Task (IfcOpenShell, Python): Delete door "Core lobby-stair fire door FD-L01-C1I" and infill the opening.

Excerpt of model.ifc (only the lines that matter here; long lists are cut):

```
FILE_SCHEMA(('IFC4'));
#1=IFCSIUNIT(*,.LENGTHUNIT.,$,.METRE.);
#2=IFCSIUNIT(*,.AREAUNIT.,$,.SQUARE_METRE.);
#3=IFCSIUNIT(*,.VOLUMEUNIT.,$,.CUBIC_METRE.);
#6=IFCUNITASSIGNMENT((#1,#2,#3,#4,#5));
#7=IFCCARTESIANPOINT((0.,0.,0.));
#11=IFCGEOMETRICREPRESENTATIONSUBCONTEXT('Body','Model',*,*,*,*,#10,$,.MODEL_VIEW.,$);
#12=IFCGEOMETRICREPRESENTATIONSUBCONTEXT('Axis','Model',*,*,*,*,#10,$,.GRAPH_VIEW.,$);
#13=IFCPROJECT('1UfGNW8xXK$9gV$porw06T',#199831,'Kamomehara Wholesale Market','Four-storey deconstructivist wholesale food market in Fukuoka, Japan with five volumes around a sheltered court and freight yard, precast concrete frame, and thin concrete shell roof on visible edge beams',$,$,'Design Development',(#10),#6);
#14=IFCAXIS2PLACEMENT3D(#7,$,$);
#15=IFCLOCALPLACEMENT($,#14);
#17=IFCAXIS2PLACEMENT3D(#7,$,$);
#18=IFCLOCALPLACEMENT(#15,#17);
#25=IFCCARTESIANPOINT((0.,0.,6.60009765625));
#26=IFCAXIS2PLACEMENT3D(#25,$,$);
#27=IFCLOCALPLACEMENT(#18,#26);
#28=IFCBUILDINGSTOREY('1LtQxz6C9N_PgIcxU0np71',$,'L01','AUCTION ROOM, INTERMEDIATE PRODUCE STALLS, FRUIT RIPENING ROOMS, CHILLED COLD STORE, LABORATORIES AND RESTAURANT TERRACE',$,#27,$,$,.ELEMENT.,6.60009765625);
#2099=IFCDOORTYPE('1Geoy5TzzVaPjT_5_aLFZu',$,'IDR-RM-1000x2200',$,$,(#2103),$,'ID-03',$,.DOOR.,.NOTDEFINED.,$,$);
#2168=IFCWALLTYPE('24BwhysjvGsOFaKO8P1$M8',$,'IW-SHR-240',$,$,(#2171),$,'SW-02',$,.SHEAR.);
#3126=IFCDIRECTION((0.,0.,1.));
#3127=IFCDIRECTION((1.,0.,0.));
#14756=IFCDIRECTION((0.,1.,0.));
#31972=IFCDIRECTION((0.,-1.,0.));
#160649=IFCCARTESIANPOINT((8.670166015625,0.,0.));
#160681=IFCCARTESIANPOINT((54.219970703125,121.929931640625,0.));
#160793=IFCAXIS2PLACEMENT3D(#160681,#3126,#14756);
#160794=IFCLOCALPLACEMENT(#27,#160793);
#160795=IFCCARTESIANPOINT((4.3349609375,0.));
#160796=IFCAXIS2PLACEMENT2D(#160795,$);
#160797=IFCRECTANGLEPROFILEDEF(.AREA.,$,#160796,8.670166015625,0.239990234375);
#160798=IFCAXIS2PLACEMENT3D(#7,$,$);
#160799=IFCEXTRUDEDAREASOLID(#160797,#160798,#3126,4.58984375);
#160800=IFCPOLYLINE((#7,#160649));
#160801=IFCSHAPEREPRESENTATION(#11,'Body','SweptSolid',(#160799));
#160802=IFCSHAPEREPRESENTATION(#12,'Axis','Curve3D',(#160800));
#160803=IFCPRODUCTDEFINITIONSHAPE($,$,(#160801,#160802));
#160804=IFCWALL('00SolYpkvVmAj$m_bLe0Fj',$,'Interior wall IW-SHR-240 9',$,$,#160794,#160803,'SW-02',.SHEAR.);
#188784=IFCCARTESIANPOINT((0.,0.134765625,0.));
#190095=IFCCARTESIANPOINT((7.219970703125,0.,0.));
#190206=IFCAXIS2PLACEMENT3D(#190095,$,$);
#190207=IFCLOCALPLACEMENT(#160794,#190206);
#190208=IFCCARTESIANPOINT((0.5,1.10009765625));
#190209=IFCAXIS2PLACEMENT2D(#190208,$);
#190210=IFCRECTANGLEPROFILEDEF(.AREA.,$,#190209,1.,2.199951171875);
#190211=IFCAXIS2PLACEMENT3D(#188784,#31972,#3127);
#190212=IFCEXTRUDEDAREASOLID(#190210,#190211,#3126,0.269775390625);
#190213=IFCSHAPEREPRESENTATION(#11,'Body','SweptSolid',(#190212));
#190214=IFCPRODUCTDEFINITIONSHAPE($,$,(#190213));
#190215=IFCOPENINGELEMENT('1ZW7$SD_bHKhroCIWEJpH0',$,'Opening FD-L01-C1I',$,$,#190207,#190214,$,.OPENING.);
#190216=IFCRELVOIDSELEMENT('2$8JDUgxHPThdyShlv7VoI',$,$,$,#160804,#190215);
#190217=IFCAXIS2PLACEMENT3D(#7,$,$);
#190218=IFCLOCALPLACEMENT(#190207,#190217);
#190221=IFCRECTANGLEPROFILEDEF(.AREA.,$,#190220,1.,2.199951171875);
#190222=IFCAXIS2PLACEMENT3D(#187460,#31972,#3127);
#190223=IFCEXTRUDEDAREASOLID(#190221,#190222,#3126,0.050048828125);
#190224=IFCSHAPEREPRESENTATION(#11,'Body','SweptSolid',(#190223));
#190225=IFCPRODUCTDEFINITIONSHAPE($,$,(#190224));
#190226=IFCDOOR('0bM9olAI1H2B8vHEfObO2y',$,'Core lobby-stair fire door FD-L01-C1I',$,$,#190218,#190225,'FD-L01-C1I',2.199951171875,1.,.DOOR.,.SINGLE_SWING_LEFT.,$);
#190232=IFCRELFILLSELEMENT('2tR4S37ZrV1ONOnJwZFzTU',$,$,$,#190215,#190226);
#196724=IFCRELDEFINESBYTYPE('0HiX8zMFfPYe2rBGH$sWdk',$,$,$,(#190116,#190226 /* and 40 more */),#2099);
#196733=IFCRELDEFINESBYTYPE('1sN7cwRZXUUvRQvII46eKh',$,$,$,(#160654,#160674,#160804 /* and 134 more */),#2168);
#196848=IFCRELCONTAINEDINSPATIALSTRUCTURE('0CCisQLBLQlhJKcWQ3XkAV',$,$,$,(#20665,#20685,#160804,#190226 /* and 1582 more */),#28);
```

```python
import ifcopenshell
import ifcopenshell.api.feature
import ifcopenshell.api.root
import ifcopenshell.geom
import ifcopenshell.util.shape

model = ifcopenshell.open("model.ifc")
settings = ifcopenshell.geom.settings()


def volume(element):
    """Net volume in cubic metres, openings subtracted."""
    shape = ifcopenshell.geom.create_shape(settings, element)
    return ifcopenshell.util.shape.get_volume(shape.geometry)


door = model.by_id(190226)
opening = door.FillsVoids[0].RelatingOpeningElement
wall = opening.VoidsElements[0].RelatingBuildingElement
before = volume(wall)

ifcopenshell.api.root.remove_product(model, product=door)
ifcopenshell.api.feature.remove_feature(model, feature=opening)

after = volume(wall)

print(f"wall volume {before:.3f} -> {after:.3f} m3")

model.write("model_edited.ifc")
```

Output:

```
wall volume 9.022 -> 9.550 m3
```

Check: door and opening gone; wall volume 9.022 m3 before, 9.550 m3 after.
